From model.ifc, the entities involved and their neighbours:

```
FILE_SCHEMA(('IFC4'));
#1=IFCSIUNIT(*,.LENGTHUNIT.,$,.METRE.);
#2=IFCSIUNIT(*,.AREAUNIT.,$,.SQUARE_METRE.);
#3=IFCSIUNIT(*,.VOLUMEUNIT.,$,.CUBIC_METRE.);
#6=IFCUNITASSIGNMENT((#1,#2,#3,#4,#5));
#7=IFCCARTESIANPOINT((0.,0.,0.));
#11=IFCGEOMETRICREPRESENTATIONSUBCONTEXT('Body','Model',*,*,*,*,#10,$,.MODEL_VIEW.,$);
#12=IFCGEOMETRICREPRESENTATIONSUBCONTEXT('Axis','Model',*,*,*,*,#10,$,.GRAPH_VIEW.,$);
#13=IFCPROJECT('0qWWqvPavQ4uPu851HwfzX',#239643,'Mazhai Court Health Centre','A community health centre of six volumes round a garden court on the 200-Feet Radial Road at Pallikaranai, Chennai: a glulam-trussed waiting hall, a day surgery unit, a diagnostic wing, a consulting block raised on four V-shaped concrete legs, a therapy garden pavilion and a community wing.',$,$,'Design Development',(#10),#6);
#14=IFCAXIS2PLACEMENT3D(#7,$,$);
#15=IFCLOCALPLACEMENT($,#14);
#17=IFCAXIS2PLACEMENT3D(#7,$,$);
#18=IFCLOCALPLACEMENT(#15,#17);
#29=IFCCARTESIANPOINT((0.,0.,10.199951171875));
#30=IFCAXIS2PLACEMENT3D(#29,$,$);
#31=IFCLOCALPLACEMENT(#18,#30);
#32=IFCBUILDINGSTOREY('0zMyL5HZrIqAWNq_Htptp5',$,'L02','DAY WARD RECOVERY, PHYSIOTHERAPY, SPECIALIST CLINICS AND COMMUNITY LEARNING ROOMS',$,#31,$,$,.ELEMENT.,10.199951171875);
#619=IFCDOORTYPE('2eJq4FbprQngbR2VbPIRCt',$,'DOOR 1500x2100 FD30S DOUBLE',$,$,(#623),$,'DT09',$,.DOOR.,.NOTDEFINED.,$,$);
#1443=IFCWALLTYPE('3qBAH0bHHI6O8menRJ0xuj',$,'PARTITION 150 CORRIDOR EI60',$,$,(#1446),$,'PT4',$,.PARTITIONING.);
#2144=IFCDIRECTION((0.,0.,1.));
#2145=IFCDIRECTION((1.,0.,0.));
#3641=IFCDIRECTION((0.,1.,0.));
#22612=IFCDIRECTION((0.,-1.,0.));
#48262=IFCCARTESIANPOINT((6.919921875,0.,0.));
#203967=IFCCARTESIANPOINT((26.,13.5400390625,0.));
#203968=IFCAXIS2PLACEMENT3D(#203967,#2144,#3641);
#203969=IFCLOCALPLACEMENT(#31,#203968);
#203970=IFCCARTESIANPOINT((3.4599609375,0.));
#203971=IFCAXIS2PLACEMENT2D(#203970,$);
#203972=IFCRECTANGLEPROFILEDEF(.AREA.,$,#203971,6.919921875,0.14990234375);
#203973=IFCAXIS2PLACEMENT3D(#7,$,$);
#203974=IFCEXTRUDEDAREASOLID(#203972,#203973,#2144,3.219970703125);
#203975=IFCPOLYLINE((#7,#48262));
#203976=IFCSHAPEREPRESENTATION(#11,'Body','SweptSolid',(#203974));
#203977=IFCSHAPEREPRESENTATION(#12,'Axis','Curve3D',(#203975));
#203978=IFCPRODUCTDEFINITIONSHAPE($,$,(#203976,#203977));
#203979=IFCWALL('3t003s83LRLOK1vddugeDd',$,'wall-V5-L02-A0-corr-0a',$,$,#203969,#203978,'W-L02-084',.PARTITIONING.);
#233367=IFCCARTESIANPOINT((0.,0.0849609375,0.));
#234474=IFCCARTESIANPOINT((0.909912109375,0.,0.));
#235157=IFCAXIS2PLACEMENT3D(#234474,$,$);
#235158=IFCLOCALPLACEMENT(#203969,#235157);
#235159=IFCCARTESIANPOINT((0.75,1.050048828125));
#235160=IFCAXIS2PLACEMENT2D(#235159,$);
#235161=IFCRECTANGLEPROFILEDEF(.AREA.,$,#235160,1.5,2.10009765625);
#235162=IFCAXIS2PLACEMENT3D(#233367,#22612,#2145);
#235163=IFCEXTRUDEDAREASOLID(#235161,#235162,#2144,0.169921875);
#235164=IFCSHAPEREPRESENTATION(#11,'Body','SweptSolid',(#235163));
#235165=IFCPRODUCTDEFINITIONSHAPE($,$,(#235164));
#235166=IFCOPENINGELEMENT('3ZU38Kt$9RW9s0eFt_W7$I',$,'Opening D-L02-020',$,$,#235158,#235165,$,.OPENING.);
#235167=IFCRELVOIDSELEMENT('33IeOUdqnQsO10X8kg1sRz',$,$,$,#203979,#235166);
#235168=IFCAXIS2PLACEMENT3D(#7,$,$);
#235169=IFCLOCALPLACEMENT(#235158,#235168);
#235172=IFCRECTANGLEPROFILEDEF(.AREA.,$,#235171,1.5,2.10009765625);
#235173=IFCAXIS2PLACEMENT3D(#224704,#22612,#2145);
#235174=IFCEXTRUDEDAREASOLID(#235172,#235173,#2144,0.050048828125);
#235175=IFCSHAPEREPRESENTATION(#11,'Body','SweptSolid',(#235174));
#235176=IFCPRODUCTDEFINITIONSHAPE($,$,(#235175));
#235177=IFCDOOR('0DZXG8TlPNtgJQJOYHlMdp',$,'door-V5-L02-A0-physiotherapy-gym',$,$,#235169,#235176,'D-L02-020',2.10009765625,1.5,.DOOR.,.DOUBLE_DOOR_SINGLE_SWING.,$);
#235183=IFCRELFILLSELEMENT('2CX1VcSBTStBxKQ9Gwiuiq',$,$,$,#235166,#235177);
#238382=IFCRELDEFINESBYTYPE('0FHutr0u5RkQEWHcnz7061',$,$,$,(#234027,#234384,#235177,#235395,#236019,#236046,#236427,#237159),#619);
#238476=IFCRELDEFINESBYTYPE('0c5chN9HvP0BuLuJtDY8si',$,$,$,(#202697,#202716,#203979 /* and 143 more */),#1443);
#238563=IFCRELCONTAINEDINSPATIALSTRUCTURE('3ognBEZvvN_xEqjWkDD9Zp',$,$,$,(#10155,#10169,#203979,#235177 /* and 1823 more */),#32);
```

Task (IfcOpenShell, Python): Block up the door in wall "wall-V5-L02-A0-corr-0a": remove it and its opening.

```python
import ifcopenshell
import ifcopenshell.api.feature
import ifcopenshell.api.root
import ifcopenshell.geom
import ifcopenshell.util.shape

model = ifcopenshell.open("model.ifc")
settings = ifcopenshell.geom.settings()


def volume(element):
    """Net volume in cubic metres, openings subtracted."""
    shape = ifcopenshell.geom.create_shape(settings, element)
    return ifcopenshell.util.shape.get_volume(shape.geometry)


door = model.by_guid("0DZXG8TlPNtgJQJOYHlMdp")
opening = door.FillsVoids[0].RelatingOpeningElement
wall = opening.VoidsElements[0].RelatingBuildingElement
before = volume(wall)

ifcopenshell.api.root.remove_product(model, product=door)
ifcopenshell.api.feature.remove_feature(model, feature=opening)

after = volume(wall)

print(f"wall volume {before:.3f} -> {after:.3f} m3")

model.write("model_rev.ifc")
```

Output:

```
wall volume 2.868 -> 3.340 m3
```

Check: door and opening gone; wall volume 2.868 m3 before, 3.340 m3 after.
